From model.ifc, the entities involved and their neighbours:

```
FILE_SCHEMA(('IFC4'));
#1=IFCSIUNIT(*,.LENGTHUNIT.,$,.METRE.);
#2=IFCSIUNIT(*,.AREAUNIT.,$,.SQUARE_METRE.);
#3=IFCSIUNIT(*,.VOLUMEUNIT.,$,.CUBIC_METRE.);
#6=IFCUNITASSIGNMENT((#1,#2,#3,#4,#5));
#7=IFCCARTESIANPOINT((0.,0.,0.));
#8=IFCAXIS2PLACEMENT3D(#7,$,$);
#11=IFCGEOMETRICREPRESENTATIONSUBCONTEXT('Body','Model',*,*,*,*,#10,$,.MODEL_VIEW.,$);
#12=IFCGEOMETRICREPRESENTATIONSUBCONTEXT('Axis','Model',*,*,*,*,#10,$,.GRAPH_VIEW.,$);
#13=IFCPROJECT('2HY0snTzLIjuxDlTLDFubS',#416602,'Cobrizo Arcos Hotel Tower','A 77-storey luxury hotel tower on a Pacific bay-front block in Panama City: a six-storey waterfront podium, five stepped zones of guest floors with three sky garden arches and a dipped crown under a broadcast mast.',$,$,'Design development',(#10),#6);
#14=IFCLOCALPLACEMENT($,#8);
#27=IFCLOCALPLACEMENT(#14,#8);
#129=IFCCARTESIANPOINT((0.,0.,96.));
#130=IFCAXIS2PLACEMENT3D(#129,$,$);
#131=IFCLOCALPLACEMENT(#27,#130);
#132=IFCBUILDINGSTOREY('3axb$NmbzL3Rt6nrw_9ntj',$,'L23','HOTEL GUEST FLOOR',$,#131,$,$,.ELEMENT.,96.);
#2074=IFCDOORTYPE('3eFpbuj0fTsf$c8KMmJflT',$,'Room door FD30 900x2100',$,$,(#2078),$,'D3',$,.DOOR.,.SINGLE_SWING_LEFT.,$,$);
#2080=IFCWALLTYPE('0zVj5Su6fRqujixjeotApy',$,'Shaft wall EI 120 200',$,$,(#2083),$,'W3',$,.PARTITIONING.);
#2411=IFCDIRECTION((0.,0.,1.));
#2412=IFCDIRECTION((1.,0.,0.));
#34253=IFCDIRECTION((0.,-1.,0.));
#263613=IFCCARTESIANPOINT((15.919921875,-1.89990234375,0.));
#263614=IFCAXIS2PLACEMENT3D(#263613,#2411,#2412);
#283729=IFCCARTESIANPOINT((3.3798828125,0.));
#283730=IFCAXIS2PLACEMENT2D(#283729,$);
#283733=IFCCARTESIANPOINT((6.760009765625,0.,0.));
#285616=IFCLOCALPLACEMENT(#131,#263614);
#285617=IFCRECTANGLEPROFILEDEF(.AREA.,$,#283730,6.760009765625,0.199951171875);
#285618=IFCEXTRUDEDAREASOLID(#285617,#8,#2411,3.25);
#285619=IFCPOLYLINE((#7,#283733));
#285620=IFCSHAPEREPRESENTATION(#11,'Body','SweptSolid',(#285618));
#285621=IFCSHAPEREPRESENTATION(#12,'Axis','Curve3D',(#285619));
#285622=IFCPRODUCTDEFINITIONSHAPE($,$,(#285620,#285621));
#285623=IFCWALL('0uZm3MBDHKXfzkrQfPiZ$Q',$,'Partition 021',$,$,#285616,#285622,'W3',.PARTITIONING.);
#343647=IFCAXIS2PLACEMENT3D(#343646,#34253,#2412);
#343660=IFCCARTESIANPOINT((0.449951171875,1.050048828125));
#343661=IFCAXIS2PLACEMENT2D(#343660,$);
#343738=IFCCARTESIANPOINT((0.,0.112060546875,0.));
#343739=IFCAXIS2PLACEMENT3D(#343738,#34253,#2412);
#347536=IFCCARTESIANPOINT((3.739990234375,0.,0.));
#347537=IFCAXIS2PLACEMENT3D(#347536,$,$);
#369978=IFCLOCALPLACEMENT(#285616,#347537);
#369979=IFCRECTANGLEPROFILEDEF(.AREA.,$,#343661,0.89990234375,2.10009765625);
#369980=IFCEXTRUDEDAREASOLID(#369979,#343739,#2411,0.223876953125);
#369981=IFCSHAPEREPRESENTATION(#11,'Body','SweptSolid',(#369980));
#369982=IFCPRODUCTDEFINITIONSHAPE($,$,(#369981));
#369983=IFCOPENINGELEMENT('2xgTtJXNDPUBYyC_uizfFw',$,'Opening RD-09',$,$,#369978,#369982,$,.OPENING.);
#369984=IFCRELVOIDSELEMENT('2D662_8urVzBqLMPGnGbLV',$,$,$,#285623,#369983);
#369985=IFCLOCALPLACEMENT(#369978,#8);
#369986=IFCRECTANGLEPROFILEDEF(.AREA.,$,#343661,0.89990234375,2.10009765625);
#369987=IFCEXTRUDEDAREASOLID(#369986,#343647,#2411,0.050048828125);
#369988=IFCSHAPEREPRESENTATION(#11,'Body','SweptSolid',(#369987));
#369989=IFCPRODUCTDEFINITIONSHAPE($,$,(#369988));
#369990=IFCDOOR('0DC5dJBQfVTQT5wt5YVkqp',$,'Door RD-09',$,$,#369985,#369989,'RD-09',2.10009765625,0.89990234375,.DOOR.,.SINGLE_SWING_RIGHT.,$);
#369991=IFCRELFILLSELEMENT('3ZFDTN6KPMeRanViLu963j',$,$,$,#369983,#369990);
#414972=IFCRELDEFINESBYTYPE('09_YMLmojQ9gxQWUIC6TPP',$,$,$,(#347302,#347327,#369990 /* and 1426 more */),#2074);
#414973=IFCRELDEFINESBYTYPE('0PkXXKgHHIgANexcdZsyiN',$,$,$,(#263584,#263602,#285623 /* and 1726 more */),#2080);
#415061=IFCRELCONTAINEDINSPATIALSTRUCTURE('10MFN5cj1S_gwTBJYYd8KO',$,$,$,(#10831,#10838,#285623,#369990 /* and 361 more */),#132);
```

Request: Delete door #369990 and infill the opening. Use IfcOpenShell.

```python
import ifcopenshell
import ifcopenshell.api.feature
import ifcopenshell.api.root
import ifcopenshell.geom
import ifcopenshell.util.shape

model = ifcopenshell.open("model.ifc")
settings = ifcopenshell.geom.settings()


def volume(element):
    """Net volume in cubic metres, openings subtracted."""
    shape = ifcopenshell.geom.create_shape(settings, element)
    return ifcopenshell.util.shape.get_volume(shape.geometry)


door = model.by_guid("0DC5dJBQfVTQT5wt5YVkqp")
opening = door.FillsVoids[0].RelatingOpeningElement
wall = opening.VoidsElements[0].RelatingBuildingElement
before = volume(wall)

ifcopenshell.api.root.remove_product(model, product=door)
ifcopenshell.api.feature.remove_feature(model, feature=opening)

after = volume(wall)

print(f"wall volume {before:.3f} -> {after:.3f} m3")

model.write("model_updated.ifc")
```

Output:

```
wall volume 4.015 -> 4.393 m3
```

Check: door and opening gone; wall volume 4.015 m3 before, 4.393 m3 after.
